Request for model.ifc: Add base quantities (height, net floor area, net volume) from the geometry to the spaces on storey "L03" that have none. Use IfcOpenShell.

First a look at what the model holds.

```python
import ifcopenshell
import ifcopenshell.util.element
import ifcopenshell.util.unit

model = ifcopenshell.open("model.ifc")
print(model.schema)
for unit_type in ("LENGTHUNIT", "AREAUNIT", "VOLUMEUNIT"):
    print(unit_type, ifcopenshell.util.unit.calculate_unit_scale(model, unit_type))
storey = next(s for s in model.by_type("IfcBuildingStorey") if s.Name == "L03")
spaces = [e for e in ifcopenshell.util.element.get_decomposition(storey) if e.is_a("IfcSpace")]
for e in sorted(spaces, key=lambda e: e.id()):
    print(e.id(), e.is_a(), e.Name, list(ifcopenshell.util.element.get_psets(e, qtos_only=True)), sep=" | ")
```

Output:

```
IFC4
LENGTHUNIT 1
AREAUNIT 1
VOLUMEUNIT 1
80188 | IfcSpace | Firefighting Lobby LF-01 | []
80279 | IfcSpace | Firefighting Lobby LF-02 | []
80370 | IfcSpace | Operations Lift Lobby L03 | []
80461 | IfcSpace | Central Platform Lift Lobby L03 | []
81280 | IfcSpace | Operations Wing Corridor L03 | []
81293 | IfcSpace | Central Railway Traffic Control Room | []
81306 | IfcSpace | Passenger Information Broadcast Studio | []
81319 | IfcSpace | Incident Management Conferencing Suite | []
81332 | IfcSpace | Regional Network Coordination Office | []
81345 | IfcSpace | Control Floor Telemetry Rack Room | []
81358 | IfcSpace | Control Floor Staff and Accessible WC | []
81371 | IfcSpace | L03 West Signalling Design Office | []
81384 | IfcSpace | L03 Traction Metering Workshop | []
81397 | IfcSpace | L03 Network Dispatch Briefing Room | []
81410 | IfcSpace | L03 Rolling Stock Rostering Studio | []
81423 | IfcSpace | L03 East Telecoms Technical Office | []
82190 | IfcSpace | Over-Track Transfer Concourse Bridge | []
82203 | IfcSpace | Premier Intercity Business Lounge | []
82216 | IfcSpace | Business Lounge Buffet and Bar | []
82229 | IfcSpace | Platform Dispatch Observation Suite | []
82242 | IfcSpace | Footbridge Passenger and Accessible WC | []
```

```python
import ifcopenshell
import ifcopenshell.api.pset
import ifcopenshell.geom
import ifcopenshell.util.element
import ifcopenshell.util.shape
import ifcopenshell.util.unit

model = ifcopenshell.open("model.ifc")
unit_scale = ifcopenshell.util.unit.calculate_unit_scale(model)
area_scale = ifcopenshell.util.unit.calculate_unit_scale(model, "AREAUNIT")
volume_scale = ifcopenshell.util.unit.calculate_unit_scale(model, "VOLUMEUNIT")
settings = ifcopenshell.geom.settings()

storey = next(s for s in model.by_type("IfcBuildingStorey") if s.Name == "L03")
spaces = [e for e in ifcopenshell.util.element.get_decomposition(storey) if e.is_a("IfcSpace")]

for e in sorted(spaces, key=lambda e: e.id()):
    if ifcopenshell.util.element.get_psets(e, qtos_only=True, should_inherit=False):
        continue
    # Geometry comes back in metres, in the element's own axes.
    shape = ifcopenshell.geom.create_shape(settings, e)
    values = {
        "Height": ifcopenshell.util.shape.get_z(shape.geometry) / unit_scale,
        "NetFloorArea": ifcopenshell.util.shape.get_footprint_area(shape.geometry) / area_scale,
        "NetVolume": ifcopenshell.util.shape.get_volume(shape.geometry) / volume_scale,
    }
    qto = ifcopenshell.api.pset.add_qto(model, product=e, name="Qto_SpaceBaseQuantities")
    ifcopenshell.api.pset.edit_qto(model, qto=qto, properties=values)
    print(e.id(), {k: round(v, 3) for k, v in values.items()})

model.write("model_edited.ifc")
```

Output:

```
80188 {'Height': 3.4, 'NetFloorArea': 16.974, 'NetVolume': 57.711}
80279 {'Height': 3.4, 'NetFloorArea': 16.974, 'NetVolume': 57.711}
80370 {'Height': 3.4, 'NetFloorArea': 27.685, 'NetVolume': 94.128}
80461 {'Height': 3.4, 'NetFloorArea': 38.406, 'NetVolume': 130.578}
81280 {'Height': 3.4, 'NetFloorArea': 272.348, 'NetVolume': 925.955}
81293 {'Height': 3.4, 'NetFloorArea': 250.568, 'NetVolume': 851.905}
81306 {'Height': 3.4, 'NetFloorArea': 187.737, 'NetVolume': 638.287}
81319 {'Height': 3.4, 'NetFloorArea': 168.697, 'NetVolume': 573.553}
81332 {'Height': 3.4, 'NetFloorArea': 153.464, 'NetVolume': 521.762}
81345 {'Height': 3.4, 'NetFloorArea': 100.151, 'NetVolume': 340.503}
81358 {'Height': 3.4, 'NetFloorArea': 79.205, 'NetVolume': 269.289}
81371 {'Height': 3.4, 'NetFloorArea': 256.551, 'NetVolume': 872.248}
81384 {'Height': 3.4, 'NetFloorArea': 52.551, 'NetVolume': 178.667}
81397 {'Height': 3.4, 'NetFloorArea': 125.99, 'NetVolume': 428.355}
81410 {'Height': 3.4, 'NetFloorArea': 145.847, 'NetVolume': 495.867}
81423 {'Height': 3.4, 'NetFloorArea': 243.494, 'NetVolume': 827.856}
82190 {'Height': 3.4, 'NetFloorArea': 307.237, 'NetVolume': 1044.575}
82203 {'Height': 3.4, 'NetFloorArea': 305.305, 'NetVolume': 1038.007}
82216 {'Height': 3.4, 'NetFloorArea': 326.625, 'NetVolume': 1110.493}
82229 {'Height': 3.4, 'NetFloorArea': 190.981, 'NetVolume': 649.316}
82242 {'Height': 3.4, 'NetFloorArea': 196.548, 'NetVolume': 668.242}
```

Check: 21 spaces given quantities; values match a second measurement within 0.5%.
